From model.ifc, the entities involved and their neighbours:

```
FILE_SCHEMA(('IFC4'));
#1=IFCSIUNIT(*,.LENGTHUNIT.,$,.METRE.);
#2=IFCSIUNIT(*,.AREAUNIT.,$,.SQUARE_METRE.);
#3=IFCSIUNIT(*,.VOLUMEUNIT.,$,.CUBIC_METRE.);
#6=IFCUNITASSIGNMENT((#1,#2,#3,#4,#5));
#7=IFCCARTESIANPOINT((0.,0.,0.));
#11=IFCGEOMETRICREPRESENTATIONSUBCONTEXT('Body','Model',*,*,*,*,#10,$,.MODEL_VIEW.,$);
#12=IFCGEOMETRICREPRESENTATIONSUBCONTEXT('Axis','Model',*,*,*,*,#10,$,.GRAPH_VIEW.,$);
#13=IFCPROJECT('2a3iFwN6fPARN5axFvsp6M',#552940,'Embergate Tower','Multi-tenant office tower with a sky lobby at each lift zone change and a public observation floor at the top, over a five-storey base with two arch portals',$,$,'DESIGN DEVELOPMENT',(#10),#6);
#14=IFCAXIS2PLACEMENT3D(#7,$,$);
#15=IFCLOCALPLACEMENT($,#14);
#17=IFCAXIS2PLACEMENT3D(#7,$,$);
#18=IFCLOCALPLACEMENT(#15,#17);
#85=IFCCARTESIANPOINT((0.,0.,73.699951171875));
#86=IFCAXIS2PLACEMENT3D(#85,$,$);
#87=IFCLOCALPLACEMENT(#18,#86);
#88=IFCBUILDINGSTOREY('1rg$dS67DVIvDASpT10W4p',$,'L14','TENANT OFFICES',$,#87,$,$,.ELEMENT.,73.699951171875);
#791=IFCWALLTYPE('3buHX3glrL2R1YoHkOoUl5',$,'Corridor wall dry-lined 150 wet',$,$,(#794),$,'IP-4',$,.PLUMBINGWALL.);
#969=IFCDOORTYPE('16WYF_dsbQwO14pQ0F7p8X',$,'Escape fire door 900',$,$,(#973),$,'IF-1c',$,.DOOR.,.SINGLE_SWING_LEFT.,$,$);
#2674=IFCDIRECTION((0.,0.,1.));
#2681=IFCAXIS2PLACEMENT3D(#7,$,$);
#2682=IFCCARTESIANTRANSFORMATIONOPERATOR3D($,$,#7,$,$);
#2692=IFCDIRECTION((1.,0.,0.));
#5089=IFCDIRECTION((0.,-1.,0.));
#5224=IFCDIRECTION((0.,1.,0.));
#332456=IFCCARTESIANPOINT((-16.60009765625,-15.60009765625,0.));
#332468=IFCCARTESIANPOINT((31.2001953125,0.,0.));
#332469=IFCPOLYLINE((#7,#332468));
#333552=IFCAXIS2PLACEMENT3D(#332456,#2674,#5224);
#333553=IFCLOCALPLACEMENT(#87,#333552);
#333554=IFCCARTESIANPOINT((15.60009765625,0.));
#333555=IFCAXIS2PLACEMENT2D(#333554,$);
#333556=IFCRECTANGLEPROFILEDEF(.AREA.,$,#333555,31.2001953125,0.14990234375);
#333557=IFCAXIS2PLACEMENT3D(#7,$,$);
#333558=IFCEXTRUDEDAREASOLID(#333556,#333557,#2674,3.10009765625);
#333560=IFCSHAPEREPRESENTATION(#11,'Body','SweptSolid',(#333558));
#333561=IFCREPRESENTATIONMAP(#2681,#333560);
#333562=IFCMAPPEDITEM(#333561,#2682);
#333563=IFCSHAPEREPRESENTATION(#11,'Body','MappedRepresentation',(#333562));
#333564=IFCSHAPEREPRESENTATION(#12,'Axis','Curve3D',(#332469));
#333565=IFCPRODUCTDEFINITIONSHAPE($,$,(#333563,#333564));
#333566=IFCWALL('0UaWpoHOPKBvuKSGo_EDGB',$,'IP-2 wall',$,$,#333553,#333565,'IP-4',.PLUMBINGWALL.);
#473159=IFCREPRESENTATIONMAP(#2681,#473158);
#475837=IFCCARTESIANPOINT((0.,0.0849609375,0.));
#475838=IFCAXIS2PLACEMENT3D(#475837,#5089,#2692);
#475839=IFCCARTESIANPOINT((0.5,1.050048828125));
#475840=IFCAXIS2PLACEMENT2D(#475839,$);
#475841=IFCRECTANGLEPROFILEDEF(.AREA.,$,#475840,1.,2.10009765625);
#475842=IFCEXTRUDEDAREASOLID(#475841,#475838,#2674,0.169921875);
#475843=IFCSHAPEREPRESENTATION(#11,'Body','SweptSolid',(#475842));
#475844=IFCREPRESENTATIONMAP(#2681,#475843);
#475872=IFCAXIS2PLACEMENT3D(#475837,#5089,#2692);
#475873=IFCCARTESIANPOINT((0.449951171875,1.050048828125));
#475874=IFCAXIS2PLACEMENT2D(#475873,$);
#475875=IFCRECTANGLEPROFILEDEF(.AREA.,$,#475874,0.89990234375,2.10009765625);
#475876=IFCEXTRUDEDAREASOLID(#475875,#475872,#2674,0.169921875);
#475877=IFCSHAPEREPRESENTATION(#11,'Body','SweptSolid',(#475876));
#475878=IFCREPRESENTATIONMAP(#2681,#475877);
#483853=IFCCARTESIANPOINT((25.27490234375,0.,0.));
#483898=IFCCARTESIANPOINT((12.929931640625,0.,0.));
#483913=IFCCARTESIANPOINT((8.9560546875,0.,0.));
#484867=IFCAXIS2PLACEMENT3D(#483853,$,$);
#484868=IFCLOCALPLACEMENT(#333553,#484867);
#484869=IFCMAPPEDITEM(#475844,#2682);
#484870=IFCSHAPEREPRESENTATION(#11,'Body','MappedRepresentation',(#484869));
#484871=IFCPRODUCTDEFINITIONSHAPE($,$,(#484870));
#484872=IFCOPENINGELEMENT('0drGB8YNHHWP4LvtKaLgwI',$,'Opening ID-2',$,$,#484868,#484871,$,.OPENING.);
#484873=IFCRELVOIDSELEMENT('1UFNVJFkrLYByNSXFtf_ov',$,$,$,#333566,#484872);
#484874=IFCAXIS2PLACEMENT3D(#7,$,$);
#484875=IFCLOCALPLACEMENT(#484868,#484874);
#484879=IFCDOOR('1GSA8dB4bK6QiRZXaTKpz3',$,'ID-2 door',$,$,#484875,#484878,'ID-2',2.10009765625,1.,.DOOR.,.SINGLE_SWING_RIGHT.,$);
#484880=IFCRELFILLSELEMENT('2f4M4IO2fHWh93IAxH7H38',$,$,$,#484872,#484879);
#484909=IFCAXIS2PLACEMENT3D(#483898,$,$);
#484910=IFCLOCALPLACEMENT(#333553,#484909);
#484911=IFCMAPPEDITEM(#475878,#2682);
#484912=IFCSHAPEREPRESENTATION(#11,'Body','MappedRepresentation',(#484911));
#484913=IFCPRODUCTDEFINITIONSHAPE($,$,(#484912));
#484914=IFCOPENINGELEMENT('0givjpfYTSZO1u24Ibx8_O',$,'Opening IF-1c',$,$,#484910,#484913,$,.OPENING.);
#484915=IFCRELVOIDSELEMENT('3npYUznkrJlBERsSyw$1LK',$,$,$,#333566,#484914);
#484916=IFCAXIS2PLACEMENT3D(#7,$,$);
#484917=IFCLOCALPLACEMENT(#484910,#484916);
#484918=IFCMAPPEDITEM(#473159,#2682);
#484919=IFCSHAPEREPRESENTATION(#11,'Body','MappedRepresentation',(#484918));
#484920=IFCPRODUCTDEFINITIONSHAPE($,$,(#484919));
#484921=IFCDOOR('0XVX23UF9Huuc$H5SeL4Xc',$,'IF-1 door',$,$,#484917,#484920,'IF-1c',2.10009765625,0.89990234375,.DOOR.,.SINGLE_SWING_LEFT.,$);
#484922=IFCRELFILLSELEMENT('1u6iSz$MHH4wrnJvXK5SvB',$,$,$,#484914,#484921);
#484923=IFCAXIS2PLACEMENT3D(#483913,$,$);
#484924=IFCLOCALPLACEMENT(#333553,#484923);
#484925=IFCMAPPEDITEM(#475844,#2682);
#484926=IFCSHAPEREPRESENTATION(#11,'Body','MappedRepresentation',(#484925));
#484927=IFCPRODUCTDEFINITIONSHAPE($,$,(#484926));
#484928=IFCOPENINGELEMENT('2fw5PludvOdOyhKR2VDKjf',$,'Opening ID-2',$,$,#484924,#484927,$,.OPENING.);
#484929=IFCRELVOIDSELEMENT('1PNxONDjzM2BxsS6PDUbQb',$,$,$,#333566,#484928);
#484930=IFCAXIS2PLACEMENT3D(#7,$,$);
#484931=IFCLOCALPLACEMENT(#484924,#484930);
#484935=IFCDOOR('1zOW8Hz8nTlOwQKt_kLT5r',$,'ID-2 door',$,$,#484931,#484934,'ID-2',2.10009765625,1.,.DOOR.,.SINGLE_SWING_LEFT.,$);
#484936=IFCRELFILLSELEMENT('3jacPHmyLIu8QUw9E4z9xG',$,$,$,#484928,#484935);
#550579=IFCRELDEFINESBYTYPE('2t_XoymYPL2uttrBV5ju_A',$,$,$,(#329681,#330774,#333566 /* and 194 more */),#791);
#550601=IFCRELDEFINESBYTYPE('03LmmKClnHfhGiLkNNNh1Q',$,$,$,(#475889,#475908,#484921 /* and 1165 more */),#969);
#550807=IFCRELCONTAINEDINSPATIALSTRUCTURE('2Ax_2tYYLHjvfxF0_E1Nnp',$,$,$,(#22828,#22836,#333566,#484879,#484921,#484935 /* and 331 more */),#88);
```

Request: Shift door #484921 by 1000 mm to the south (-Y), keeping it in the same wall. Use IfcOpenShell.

```python
import ifcopenshell
import ifcopenshell.api.geometry
import ifcopenshell.util.placement
import ifcopenshell.util.unit

model = ifcopenshell.open("model.ifc")
unit_scale = ifcopenshell.util.unit.calculate_unit_scale(model)

door = model.by_id(484921)
opening = door.FillsVoids[0].RelatingOpeningElement
wall = opening.VoidsElements[0].RelatingBuildingElement

wall_matrix = ifcopenshell.util.placement.get_local_placement(wall.ObjectPlacement)
shift = wall_matrix[:3, 0] * -1 / unit_scale
before = ifcopenshell.util.placement.get_local_placement(door.ObjectPlacement)[:3, 3].copy()

# The door is placed relative to its opening, so it follows when the opening moves.
matrix = ifcopenshell.util.placement.get_local_placement(opening.ObjectPlacement)
matrix[:3, 3] += shift
ifcopenshell.api.geometry.edit_object_placement(
    model, product=opening, matrix=matrix, is_si=False, should_transform_children=True
)

after = ifcopenshell.util.placement.get_local_placement(door.ObjectPlacement)[:3, 3]
print("door moved by", (after - before).round(3) + 0.0)

model.write("model-out.ifc")
```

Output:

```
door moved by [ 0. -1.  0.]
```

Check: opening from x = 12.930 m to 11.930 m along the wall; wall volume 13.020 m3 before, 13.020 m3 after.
